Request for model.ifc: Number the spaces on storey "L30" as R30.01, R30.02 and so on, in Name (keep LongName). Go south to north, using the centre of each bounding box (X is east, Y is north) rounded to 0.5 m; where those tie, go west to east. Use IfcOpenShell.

First a look at what the model holds.

```python
import ifcopenshell
import ifcopenshell.util.element
import ifcopenshell.util.placement

model = ifcopenshell.open("model.ifc")
print(model.schema)
storey = next(s for s in model.by_type("IfcBuildingStorey") if s.Name == "L30")
spaces = [e for e in ifcopenshell.util.element.get_decomposition(storey) if e.is_a("IfcSpace")]
for e in sorted(spaces, key=lambda e: e.id()):
    origin = ifcopenshell.util.placement.get_local_placement(e.ObjectPlacement)[:3, 3]
    print(e.id(), e.Name, e.LongName, origin.round(2) + 0.0, sep=" | ")
```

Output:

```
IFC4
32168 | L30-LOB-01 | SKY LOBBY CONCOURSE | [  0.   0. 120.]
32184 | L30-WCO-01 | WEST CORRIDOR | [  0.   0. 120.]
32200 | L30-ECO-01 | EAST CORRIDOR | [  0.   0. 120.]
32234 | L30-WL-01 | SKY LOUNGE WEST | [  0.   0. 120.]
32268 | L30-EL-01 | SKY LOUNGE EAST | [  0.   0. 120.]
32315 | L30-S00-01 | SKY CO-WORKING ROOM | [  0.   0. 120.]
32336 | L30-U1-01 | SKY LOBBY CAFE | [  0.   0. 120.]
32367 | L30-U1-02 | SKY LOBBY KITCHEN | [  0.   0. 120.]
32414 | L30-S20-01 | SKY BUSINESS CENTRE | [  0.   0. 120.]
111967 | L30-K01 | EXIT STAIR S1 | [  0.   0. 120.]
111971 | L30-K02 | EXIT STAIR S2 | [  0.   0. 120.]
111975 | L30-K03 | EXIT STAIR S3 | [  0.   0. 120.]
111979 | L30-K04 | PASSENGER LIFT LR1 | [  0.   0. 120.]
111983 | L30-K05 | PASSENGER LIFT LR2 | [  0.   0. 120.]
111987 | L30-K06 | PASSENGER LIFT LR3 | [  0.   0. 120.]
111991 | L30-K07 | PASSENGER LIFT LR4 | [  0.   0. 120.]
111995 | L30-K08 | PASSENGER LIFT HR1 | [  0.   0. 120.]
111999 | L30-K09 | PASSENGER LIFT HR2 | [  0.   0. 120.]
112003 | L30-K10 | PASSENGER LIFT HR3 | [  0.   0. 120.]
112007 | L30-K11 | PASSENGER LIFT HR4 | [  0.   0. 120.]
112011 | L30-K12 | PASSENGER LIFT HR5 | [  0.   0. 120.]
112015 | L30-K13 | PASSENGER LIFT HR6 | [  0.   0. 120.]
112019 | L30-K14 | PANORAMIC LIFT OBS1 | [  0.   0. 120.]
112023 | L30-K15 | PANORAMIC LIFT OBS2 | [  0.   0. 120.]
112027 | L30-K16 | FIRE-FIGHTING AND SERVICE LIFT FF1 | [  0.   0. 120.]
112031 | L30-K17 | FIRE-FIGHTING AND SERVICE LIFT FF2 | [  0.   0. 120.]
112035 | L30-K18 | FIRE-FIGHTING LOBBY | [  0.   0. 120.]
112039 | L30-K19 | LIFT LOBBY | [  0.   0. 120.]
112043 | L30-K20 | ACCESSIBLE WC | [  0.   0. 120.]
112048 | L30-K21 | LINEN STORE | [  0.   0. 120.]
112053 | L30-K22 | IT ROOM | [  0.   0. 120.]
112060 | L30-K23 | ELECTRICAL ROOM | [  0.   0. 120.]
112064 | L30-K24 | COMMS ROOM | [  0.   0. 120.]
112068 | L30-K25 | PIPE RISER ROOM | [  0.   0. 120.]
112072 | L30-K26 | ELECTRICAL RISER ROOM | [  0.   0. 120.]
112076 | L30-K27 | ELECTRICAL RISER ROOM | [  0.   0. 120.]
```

```python
import ifcopenshell
import ifcopenshell.geom
import ifcopenshell.util.element
import ifcopenshell.util.shape

model = ifcopenshell.open("model.ifc")
settings = ifcopenshell.geom.settings()
settings.set("use-world-coords", True)


def centre(element):
    shape = ifcopenshell.geom.create_shape(settings, element)
    return ifcopenshell.util.shape.get_bbox_centroid(shape.geometry)


storey = next(s for s in model.by_type("IfcBuildingStorey") if s.Name == "L30")
spaces = [e for e in ifcopenshell.util.element.get_decomposition(storey) if e.is_a("IfcSpace")]

# Insertion points can sit at a corner or the storey origin, so sort by the geometry (in metres).
centres = {e: centre(e) for e in spaces}
spaces.sort(key=lambda e: (round(centres[e][1] / 0.5), centres[e][0]))

for i, e in enumerate(spaces, start=1):
    number = f"R30.{i:02d}"
    e.Name = number
    print(e.id(), number)

model.write("model_edited.ifc")
```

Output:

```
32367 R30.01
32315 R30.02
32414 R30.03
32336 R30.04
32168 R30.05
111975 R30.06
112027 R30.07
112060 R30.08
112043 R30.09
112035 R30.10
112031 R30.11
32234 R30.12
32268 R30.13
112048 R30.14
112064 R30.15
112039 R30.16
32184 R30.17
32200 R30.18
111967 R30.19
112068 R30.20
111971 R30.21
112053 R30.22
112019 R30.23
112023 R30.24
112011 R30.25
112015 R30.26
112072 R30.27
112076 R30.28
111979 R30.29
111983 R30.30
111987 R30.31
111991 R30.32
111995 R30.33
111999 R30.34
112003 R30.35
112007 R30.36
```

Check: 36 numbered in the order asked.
